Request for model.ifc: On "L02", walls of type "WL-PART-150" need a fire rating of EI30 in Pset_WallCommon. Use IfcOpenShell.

First a look at what the model holds.

```python
import ifcopenshell
import ifcopenshell.util.element

model = ifcopenshell.open("model.ifc")
print(model.schema)
storey = next(s for s in model.by_type("IfcBuildingStorey") if s.Name == "L02")
walls = [e for e in ifcopenshell.util.element.get_decomposition(storey) if e.is_a("IfcWall")]
seen = {}
for e in walls:
    element_type = ifcopenshell.util.element.get_type(e)
    key = (element_type.Name if element_type != e and element_type else None, ifcopenshell.util.element.get_pset(e, "Pset_WallCommon", "FireRating"))
    seen[key] = seen.get(key, 0) + 1
for (name, value), count in sorted(seen.items(), key=str):
    print(count, "x", name, "|", value)
```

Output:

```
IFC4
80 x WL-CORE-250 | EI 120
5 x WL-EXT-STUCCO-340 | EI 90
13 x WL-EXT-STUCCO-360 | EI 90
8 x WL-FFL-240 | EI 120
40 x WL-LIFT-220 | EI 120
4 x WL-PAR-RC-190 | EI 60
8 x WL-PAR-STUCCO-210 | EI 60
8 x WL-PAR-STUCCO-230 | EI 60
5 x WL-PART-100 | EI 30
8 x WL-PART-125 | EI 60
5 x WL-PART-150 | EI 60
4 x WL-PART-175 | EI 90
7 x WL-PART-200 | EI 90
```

```python
import ifcopenshell
import ifcopenshell.api.pset
import ifcopenshell.util.element

model = ifcopenshell.open("model.ifc")

storey = next(s for s in model.by_type("IfcBuildingStorey") if s.Name == "L02")
walls = [e for e in ifcopenshell.util.element.get_decomposition(storey) if e.is_a("IfcWall")]

count = 0
for e in walls:
    element_type = ifcopenshell.util.element.get_type(e)
    if element_type in (None, e) or element_type.Name != "WL-PART-150":
        continue
    # add_pset returns the element's existing set when there is one.
    pset = ifcopenshell.api.pset.add_pset(model, product=e, name="Pset_WallCommon")
    ifcopenshell.api.pset.edit_pset(model, pset=pset, properties={"FireRating": "EI30"})
    count += 1

print(count, "walls updated")

model.write("model_edited.ifc")
```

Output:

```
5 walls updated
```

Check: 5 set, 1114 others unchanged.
